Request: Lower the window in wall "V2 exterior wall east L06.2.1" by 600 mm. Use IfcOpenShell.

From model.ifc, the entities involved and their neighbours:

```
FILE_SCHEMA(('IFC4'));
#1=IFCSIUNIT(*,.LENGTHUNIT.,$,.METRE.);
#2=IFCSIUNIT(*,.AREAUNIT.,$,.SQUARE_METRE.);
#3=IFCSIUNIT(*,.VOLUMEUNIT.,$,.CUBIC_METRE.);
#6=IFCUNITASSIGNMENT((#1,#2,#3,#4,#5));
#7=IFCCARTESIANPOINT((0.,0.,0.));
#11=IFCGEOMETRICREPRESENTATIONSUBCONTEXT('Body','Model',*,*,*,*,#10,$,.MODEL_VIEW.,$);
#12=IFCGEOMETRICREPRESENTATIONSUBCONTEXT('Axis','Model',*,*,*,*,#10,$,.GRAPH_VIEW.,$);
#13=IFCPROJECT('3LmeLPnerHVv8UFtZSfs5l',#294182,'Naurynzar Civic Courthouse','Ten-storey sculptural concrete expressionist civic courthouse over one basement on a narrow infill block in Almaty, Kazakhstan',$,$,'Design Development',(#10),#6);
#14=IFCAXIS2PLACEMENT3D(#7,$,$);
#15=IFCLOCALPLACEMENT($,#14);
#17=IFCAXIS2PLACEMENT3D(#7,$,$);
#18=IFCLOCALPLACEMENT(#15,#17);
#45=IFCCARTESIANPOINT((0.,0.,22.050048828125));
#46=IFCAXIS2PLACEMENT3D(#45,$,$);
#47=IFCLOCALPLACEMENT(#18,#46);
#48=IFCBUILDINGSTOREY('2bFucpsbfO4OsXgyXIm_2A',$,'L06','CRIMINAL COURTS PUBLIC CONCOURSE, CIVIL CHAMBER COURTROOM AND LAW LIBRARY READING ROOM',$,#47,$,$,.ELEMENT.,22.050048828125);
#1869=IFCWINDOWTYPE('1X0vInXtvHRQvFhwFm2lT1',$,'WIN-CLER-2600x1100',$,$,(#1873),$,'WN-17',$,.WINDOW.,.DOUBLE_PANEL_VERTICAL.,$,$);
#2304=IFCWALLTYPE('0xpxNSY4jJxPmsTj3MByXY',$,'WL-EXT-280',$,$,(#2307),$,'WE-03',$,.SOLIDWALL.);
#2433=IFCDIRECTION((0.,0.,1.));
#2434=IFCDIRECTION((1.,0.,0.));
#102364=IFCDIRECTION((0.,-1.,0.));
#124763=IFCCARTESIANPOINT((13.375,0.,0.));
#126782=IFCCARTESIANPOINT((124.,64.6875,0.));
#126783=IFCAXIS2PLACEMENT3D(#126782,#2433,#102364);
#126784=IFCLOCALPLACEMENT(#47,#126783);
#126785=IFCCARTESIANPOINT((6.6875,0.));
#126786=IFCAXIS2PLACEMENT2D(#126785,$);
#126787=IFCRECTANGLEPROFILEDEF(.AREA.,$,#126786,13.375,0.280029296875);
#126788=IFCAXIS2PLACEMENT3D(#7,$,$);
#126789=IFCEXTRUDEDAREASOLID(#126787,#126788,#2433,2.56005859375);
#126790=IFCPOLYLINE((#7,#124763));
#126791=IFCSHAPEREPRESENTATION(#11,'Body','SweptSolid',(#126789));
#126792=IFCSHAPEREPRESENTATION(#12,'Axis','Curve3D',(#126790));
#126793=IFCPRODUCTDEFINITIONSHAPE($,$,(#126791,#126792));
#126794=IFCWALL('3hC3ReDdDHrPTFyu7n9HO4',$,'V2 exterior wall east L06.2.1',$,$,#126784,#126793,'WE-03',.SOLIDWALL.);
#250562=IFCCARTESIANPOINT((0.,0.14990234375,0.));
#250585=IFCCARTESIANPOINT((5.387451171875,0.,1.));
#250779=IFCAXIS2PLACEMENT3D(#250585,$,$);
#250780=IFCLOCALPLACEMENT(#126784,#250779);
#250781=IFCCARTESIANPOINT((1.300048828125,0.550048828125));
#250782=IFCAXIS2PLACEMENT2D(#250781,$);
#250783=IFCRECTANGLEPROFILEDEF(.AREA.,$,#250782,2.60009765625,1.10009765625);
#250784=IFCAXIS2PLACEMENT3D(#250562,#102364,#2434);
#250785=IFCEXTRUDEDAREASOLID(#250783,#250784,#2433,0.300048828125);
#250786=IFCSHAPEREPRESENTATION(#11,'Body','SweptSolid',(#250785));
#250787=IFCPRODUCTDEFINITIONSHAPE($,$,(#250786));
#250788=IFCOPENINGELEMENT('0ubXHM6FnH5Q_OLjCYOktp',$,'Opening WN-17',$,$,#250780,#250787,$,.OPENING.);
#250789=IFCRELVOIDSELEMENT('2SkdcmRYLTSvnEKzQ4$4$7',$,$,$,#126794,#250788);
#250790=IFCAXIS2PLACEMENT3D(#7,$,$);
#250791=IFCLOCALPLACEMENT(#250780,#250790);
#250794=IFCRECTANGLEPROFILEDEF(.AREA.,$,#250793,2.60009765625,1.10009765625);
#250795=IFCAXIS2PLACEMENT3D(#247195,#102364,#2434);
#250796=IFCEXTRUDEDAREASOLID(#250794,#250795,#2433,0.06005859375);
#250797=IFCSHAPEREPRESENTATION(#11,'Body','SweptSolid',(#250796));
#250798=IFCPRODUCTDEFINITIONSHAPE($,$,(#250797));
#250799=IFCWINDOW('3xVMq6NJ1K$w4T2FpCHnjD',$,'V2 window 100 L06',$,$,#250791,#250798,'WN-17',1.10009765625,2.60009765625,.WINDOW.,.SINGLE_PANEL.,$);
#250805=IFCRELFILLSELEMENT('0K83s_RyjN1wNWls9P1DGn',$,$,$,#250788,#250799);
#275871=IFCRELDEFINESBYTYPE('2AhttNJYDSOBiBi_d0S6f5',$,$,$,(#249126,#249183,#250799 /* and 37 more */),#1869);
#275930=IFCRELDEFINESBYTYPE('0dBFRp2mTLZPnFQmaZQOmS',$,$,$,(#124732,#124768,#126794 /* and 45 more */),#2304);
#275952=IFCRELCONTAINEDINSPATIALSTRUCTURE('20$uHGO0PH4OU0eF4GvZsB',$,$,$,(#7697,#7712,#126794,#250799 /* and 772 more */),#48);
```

```python
import numpy as np
import ifcopenshell
import ifcopenshell.api.geometry
import ifcopenshell.util.placement
import ifcopenshell.util.unit

model = ifcopenshell.open("model.ifc")
unit_scale = ifcopenshell.util.unit.calculate_unit_scale(model)

window = model.by_guid("3xVMq6NJ1K$w4T2FpCHnjD")
opening = window.FillsVoids[0].RelatingOpeningElement
dz = -0.6

shift = np.array([0.0, 0.0, dz])
# The window is placed relative to its opening, so it follows when the opening moves.
matrix = ifcopenshell.util.placement.get_local_placement(opening.ObjectPlacement)
matrix[:3, 3] += shift
ifcopenshell.api.geometry.edit_object_placement(
    model, product=opening, matrix=matrix, is_si=False, should_transform_children=True
)

print(f"moved by {dz * unit_scale:+.3f} m")

model.write("model_edited.ifc")
```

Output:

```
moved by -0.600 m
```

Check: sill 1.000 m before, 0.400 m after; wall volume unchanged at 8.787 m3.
